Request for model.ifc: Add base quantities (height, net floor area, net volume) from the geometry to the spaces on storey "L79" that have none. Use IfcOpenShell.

First a look at what the model holds.

```python
import ifcopenshell
import ifcopenshell.util.element
import ifcopenshell.util.unit

model = ifcopenshell.open("model.ifc")
print(model.schema)
for unit_type in ("LENGTHUNIT", "AREAUNIT", "VOLUMEUNIT"):
    print(unit_type, ifcopenshell.util.unit.calculate_unit_scale(model, unit_type))
storey = next(s for s in model.by_type("IfcBuildingStorey") if s.Name == "L79")
spaces = [e for e in ifcopenshell.util.element.get_decomposition(storey) if e.is_a("IfcSpace")]
for e in sorted(spaces, key=lambda e: e.id()):
    print(e.id(), e.is_a(), e.Name, list(ifcopenshell.util.element.get_psets(e, qtos_only=True)), sep=" | ")
```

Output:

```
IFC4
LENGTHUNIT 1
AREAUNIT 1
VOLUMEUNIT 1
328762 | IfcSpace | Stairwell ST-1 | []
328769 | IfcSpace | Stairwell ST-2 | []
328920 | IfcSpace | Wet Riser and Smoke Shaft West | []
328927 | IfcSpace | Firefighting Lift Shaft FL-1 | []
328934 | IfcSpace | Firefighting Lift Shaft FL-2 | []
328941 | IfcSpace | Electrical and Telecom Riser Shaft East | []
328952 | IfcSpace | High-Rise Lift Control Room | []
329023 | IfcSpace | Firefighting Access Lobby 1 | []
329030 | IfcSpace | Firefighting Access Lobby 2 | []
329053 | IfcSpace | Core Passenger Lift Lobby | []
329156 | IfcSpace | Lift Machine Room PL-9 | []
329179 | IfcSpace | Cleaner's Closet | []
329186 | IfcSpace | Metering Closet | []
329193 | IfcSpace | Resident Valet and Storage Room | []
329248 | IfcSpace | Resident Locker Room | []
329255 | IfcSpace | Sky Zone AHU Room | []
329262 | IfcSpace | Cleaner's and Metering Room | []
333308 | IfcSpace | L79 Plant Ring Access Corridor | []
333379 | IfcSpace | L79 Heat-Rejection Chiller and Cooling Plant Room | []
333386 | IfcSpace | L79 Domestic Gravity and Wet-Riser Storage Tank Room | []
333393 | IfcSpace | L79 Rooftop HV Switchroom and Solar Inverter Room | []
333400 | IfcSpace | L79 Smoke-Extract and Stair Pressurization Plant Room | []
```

```python
import ifcopenshell
import ifcopenshell.api.pset
import ifcopenshell.geom
import ifcopenshell.util.element
import ifcopenshell.util.shape
import ifcopenshell.util.unit

model = ifcopenshell.open("model.ifc")
unit_scale = ifcopenshell.util.unit.calculate_unit_scale(model)
area_scale = ifcopenshell.util.unit.calculate_unit_scale(model, "AREAUNIT")
volume_scale = ifcopenshell.util.unit.calculate_unit_scale(model, "VOLUMEUNIT")
settings = ifcopenshell.geom.settings()

storey = next(s for s in model.by_type("IfcBuildingStorey") if s.Name == "L79")
spaces = [e for e in ifcopenshell.util.element.get_decomposition(storey) if e.is_a("IfcSpace")]

for e in sorted(spaces, key=lambda e: e.id()):
    if ifcopenshell.util.element.get_psets(e, qtos_only=True, should_inherit=False):
        continue
    # Geometry comes back in metres, in the element's own axes.
    shape = ifcopenshell.geom.create_shape(settings, e)
    values = {
        "Height": ifcopenshell.util.shape.get_z(shape.geometry) / unit_scale,
        "NetFloorArea": ifcopenshell.util.shape.get_footprint_area(shape.geometry) / area_scale,
        "NetVolume": ifcopenshell.util.shape.get_volume(shape.geometry) / volume_scale,
    }
    qto = ifcopenshell.api.pset.add_qto(model, product=e, name="Qto_SpaceBaseQuantities")
    ifcopenshell.api.pset.edit_qto(model, qto=qto, properties=values)
    print(e.id(), {k: round(v, 3) for k, v in values.items()})

model.write("model_updated.ifc")
```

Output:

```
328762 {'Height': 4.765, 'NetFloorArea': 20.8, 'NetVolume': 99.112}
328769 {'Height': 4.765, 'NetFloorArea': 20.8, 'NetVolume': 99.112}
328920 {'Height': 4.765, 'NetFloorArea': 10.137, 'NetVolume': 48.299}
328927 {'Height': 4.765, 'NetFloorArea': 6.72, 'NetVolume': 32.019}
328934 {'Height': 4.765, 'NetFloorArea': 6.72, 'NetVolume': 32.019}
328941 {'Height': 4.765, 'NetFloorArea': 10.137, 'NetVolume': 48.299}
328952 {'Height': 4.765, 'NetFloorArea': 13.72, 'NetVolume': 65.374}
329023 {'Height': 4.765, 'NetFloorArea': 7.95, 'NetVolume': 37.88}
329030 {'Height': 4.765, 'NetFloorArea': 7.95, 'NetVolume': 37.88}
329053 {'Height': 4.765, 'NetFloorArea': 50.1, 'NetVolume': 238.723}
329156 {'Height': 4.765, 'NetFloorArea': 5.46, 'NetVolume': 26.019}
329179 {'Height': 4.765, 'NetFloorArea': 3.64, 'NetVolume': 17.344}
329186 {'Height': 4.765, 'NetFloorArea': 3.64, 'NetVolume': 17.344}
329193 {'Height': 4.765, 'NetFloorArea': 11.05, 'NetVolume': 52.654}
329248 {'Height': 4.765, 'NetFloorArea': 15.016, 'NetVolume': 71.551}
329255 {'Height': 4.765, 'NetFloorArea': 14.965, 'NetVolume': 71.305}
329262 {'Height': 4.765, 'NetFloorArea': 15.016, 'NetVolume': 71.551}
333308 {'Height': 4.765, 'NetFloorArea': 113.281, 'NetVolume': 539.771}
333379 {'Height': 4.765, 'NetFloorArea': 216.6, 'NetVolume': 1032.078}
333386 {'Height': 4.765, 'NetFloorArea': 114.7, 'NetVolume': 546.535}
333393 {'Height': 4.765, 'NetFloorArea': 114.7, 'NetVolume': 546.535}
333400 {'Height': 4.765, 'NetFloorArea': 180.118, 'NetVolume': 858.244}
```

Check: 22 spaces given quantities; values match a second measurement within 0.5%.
